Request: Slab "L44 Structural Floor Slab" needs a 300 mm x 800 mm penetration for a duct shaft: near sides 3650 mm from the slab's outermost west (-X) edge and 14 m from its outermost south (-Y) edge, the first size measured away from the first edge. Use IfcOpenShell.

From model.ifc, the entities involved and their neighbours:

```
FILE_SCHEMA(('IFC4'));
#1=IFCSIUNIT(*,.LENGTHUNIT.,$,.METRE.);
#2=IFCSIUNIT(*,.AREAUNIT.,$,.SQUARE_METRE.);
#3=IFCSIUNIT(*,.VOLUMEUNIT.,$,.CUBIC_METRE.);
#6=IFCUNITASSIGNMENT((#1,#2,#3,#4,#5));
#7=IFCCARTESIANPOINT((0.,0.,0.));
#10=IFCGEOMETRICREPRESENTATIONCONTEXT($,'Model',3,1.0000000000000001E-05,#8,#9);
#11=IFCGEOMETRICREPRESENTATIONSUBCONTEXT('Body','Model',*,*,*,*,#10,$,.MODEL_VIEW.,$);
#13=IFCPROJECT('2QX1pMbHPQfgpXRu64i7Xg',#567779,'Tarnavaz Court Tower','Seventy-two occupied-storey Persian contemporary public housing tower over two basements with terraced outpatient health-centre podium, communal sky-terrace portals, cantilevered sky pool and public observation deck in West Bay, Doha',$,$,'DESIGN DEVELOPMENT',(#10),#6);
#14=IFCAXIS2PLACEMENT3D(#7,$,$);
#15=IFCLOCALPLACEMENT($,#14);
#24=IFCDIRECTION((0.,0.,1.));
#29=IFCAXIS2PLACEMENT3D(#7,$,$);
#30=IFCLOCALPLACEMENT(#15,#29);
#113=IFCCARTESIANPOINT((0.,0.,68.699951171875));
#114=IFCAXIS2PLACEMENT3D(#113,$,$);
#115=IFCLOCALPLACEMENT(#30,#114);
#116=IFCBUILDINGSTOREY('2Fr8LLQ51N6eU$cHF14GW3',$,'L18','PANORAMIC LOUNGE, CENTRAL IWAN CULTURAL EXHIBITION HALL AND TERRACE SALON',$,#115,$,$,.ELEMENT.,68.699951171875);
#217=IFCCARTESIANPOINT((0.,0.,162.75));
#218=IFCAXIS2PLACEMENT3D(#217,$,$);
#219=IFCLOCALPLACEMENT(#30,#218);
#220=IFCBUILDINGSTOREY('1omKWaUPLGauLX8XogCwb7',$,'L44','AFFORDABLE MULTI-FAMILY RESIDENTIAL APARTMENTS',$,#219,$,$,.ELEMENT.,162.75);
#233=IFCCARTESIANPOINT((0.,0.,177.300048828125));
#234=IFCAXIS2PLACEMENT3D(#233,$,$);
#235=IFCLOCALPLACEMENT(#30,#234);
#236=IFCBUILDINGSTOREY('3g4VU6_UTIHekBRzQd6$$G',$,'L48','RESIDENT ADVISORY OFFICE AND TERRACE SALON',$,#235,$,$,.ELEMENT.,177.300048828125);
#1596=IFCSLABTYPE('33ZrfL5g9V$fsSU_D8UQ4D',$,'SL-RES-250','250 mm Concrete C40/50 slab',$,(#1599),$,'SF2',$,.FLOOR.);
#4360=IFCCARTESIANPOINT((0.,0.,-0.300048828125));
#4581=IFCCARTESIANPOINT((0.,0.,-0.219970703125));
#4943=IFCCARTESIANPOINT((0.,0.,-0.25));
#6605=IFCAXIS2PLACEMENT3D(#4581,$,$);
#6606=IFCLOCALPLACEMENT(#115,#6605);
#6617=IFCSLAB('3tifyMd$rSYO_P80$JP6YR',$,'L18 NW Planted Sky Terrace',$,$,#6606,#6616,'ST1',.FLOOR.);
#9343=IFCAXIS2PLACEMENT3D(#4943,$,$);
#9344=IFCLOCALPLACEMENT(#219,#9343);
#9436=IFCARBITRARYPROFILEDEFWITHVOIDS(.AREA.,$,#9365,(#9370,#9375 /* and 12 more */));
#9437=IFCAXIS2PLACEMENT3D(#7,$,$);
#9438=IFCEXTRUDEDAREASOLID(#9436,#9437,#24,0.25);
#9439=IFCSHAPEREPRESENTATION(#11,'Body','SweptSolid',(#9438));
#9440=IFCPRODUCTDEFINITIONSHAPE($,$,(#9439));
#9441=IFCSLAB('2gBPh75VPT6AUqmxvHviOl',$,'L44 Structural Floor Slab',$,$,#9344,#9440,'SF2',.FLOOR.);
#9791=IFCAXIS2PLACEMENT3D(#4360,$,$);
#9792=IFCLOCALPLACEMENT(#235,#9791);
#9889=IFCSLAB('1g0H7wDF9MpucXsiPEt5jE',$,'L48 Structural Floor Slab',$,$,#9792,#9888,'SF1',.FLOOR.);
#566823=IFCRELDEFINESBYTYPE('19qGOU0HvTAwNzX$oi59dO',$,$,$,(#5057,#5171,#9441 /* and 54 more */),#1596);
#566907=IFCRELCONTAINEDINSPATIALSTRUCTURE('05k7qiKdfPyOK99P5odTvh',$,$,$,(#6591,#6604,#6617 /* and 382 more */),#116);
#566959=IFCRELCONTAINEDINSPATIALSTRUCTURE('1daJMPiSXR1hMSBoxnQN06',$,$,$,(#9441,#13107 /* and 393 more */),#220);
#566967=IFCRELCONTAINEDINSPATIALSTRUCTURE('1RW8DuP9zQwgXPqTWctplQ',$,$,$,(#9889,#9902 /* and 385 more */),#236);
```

```python
import numpy as np
import ifcopenshell
import ifcopenshell.api.feature
import ifcopenshell.api.geometry
import ifcopenshell.api.root
import ifcopenshell.geom
import ifcopenshell.util.placement
import ifcopenshell.util.representation
import ifcopenshell.util.shape
import ifcopenshell.util.unit

model = ifcopenshell.open("model.ifc")
unit_scale = ifcopenshell.util.unit.calculate_unit_scale(model)
settings = ifcopenshell.geom.settings()


def volume(element):
    """Net volume in cubic metres, openings subtracted."""
    shape = ifcopenshell.geom.create_shape(settings, element)
    return ifcopenshell.util.shape.get_volume(shape.geometry)


slab = model.by_id(9441)
before = volume(slab)

# Extent in the slab's own axes, in metres. The edges named are its -X and -Y sides.
slab_shape = ifcopenshell.geom.create_shape(settings, slab)
vertices = ifcopenshell.util.shape.get_vertices(slab_shape.geometry)
x_min, y_min, bottom = vertices.min(axis=0)
top = vertices[:, 2].max()

opening = ifcopenshell.api.root.create_entity(model, ifc_class="IfcOpeningElement", name="Duct shaft opening", predefined_type="OPENING")
context = ifcopenshell.util.representation.get_context(model, "Model", "Body", "MODEL_VIEW")
width, depth = 0.3, 0.8
outline = [(0.0, 0.0), (width, 0.0), (width, depth), (0.0, depth), (0.0, 0.0)]
# Overshoot both faces by 50 mm so the cut is clean.
shape = ifcopenshell.api.geometry.add_slab_representation(
    model, context=context, depth=top - bottom + 0.1, polyline=outline
)
ifcopenshell.api.geometry.assign_representation(model, product=opening, representation=shape)

matrix = ifcopenshell.util.placement.get_local_placement(slab.ObjectPlacement)
matrix[:, 3] = matrix @ np.append(np.array([x_min + 3.65, y_min + 14, bottom - 0.05]) / unit_scale, 1.0)
ifcopenshell.api.geometry.edit_object_placement(model, product=opening, matrix=matrix, is_si=False)
ifcopenshell.api.feature.add_feature(model, feature=opening, element=slab)

after = volume(slab)

print(f"slab volume {before:.3f} -> {after:.3f} m3")

model.write("model_rev.ifc")
```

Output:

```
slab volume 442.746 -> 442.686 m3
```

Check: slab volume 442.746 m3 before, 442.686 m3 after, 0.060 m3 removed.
